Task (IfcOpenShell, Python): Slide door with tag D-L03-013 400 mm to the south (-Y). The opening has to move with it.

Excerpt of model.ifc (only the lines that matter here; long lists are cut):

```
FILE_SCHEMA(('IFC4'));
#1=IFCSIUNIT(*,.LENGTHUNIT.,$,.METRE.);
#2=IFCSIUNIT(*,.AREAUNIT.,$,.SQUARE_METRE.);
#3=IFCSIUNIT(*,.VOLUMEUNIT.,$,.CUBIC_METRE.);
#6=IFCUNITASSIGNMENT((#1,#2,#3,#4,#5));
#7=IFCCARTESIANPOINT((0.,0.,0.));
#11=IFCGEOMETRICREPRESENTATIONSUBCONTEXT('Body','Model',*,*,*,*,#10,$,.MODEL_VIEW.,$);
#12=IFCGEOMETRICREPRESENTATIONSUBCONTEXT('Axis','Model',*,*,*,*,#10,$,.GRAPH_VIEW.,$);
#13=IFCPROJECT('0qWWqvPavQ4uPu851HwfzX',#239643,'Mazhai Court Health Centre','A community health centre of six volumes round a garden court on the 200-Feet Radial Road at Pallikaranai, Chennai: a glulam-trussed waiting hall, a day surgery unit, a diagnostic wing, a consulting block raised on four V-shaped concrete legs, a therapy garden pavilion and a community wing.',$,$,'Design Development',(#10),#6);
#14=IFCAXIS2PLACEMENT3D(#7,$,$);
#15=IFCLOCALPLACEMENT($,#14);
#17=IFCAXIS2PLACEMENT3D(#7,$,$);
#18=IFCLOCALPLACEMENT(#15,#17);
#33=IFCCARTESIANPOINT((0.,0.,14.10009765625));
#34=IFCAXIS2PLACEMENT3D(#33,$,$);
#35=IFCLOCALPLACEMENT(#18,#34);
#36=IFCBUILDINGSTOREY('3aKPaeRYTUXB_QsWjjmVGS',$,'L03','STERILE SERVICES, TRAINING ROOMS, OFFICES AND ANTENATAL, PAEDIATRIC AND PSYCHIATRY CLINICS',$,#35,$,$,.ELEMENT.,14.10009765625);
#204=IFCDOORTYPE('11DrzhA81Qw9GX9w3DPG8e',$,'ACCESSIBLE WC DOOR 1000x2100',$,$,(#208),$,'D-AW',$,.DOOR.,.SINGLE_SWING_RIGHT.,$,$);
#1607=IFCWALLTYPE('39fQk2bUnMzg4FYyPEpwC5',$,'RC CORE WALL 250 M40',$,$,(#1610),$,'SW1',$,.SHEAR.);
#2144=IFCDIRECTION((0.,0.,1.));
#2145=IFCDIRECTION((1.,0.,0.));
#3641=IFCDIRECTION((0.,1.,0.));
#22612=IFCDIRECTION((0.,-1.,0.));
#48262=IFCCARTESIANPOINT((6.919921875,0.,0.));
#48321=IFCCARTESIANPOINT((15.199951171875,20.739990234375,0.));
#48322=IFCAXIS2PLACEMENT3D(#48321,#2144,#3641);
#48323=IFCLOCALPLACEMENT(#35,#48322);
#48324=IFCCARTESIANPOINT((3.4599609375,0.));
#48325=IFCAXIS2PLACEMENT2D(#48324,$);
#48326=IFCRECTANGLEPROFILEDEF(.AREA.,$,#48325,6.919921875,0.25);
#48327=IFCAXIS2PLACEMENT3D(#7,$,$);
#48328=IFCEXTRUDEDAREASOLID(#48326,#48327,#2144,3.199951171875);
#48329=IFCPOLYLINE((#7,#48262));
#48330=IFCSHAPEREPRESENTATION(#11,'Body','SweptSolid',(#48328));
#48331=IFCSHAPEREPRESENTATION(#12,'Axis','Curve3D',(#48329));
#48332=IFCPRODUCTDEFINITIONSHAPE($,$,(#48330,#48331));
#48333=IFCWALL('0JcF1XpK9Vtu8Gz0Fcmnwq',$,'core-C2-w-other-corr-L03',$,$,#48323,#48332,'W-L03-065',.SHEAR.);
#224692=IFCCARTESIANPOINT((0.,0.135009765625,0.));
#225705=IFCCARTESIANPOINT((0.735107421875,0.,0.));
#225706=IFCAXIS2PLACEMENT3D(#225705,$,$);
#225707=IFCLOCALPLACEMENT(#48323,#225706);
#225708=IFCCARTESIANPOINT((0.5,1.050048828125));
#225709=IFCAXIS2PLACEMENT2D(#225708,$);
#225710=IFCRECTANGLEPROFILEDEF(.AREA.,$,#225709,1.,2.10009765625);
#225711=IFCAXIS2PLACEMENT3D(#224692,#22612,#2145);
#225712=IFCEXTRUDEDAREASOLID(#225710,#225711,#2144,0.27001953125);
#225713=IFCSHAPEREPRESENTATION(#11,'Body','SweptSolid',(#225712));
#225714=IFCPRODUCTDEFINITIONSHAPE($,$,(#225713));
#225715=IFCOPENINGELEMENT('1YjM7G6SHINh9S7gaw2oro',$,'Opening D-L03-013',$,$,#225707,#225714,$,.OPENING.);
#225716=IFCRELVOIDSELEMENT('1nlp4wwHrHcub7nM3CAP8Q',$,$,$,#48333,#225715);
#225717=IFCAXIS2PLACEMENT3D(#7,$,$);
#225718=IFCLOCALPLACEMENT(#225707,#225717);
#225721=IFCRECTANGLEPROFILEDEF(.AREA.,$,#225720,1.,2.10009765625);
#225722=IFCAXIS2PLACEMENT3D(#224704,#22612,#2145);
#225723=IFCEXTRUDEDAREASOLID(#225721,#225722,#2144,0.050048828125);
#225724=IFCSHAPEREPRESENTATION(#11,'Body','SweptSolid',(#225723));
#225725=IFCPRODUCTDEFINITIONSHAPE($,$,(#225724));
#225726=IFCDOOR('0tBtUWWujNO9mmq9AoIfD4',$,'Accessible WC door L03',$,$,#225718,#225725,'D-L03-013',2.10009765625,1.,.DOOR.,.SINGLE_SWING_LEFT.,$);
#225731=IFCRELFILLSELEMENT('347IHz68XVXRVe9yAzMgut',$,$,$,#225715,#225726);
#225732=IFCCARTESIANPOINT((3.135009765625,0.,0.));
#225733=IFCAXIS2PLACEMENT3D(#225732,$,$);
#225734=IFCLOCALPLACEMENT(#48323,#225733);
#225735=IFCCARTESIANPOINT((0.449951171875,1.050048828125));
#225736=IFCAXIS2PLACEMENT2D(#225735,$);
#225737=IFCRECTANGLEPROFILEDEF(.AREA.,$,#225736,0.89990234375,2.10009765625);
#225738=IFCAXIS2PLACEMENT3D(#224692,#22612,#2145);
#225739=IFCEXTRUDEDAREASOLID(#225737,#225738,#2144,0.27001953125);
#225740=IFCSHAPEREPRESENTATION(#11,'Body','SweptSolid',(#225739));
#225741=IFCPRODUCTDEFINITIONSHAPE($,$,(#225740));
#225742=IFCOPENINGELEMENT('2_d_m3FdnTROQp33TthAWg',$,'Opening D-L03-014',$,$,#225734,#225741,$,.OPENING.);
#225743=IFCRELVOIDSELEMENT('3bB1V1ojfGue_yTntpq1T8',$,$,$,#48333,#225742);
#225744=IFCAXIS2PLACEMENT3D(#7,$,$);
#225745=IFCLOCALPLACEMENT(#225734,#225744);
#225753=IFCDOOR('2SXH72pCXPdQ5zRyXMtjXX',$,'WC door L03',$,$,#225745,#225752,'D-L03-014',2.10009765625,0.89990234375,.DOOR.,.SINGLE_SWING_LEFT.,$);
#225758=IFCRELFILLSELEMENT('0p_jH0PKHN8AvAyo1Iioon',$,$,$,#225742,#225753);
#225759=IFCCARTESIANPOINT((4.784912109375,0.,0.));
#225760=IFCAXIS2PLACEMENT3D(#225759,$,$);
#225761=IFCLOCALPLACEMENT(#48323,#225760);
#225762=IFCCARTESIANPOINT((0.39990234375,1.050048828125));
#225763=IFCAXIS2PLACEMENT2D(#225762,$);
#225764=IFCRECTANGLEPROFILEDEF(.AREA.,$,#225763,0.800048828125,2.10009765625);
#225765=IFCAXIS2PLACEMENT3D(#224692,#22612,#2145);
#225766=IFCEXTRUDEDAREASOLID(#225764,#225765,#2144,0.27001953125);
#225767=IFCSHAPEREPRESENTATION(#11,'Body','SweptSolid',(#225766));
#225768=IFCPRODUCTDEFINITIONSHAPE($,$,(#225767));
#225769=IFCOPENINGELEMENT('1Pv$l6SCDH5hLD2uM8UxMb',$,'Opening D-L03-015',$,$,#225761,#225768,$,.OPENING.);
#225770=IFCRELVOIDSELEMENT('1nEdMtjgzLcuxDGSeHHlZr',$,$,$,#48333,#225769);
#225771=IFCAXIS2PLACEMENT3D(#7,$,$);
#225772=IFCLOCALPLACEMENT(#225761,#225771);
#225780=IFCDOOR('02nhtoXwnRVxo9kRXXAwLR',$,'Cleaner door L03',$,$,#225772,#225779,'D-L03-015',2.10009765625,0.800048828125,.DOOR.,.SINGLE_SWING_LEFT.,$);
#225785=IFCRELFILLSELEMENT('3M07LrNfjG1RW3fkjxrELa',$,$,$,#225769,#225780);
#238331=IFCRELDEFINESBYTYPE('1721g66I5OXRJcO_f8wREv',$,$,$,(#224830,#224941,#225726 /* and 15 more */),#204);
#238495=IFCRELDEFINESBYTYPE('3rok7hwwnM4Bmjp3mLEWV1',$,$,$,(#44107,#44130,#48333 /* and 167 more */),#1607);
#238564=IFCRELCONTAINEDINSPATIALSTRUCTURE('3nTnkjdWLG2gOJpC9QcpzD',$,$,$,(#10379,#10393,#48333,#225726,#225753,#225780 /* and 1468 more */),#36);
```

```python
import ifcopenshell
import ifcopenshell.api.geometry
import ifcopenshell.util.placement

model = ifcopenshell.open("model.ifc")

door = model.by_guid("0tBtUWWujNO9mmq9AoIfD4")
opening = door.FillsVoids[0].RelatingOpeningElement
wall = opening.VoidsElements[0].RelatingBuildingElement

wall_matrix = ifcopenshell.util.placement.get_local_placement(wall.ObjectPlacement)
shift = wall_matrix[:3, 0] * -0.4
before = ifcopenshell.util.placement.get_local_placement(door.ObjectPlacement)[:3, 3].copy()

# The door is placed relative to its opening, so it follows when the opening moves.
matrix = ifcopenshell.util.placement.get_local_placement(opening.ObjectPlacement)
matrix[:3, 3] += shift
ifcopenshell.api.geometry.edit_object_placement(
    model, product=opening, matrix=matrix, is_si=False, should_transform_children=True
)

after = ifcopenshell.util.placement.get_local_placement(door.ObjectPlacement)[:3, 3]
print("door moved by", (after - before).round(3) + 0.0)

model.write("model_updated.ifc")
```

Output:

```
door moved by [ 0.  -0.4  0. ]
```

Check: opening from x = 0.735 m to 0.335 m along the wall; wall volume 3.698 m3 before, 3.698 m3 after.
